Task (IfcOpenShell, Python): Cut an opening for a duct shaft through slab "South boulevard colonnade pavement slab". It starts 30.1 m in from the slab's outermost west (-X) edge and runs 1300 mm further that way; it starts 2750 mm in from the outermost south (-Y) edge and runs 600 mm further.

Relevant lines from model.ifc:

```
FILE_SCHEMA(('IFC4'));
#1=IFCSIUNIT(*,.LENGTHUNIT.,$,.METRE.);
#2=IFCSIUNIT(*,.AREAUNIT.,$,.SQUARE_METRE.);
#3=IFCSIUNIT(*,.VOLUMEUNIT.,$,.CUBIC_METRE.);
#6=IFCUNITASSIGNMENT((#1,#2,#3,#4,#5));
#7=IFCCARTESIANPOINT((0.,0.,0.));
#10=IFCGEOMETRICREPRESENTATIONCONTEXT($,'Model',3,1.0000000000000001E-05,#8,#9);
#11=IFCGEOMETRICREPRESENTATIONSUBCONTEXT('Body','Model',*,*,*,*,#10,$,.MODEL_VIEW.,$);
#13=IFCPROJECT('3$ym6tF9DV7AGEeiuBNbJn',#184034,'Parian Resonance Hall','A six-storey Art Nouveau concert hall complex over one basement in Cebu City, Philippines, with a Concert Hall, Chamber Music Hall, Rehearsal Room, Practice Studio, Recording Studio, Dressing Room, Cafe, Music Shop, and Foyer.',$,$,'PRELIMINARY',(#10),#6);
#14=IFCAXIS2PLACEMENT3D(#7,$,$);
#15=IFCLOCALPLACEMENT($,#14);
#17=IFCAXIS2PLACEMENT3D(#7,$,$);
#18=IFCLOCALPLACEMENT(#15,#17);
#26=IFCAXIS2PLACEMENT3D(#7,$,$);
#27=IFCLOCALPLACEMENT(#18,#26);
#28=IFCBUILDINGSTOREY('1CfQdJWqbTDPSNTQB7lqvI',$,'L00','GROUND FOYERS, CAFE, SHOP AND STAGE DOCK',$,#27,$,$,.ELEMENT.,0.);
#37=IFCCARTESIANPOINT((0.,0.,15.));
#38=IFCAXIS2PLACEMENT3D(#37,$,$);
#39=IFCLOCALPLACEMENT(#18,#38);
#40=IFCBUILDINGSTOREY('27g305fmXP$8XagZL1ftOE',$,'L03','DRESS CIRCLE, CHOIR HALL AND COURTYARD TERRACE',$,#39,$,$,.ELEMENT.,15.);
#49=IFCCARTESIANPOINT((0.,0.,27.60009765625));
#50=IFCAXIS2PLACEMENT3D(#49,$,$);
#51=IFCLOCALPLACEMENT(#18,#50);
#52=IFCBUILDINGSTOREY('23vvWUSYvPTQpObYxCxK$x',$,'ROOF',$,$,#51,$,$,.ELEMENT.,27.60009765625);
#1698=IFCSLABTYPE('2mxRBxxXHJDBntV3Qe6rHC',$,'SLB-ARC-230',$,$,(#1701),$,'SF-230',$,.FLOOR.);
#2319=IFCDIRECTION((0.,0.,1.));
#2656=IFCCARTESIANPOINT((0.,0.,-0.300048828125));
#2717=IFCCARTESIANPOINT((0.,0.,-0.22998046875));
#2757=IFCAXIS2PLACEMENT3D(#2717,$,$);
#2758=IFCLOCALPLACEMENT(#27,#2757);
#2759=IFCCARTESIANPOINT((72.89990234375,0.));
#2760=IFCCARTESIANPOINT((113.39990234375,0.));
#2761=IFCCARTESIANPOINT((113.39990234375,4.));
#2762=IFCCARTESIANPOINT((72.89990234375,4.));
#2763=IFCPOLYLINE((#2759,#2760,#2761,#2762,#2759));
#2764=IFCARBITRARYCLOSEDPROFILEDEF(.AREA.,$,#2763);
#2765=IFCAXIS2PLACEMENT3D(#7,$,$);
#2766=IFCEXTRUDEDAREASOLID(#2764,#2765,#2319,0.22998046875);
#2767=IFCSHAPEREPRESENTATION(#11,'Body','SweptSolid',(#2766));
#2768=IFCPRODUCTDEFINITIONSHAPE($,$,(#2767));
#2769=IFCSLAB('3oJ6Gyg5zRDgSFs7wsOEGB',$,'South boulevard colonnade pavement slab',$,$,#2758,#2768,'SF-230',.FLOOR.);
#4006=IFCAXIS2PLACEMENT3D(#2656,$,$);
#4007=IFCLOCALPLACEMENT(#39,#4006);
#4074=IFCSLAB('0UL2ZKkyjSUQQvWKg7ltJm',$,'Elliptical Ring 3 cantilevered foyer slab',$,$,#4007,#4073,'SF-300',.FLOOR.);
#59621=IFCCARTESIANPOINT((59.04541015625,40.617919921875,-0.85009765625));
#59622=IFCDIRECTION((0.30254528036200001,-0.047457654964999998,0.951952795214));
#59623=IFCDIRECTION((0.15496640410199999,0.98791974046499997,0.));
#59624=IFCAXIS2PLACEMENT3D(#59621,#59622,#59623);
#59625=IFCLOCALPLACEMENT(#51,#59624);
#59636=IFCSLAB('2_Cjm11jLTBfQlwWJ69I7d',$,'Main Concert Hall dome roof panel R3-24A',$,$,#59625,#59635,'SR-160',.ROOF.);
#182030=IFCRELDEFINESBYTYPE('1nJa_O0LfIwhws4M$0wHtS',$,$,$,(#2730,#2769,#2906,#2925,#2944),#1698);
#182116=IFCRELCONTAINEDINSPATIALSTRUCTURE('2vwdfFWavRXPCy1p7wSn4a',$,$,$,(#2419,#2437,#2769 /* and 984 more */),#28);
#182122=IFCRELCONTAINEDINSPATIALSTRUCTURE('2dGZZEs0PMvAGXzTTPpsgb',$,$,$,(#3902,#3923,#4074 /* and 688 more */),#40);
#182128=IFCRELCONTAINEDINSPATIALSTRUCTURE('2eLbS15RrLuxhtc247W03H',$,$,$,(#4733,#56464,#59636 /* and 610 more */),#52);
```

```python
import numpy as np
import ifcopenshell
import ifcopenshell.api.feature
import ifcopenshell.api.geometry
import ifcopenshell.api.root
import ifcopenshell.geom
import ifcopenshell.util.placement
import ifcopenshell.util.representation
import ifcopenshell.util.shape
import ifcopenshell.util.unit

model = ifcopenshell.open("model.ifc")
unit_scale = ifcopenshell.util.unit.calculate_unit_scale(model)
settings = ifcopenshell.geom.settings()


def volume(element):
    """Net volume in cubic metres, openings subtracted."""
    shape = ifcopenshell.geom.create_shape(settings, element)
    return ifcopenshell.util.shape.get_volume(shape.geometry)


slab = model.by_guid("3oJ6Gyg5zRDgSFs7wsOEGB")
before = volume(slab)

# Extent in the slab's own axes, in metres. The edges named are its -X and -Y sides.
slab_shape = ifcopenshell.geom.create_shape(settings, slab)
vertices = ifcopenshell.util.shape.get_vertices(slab_shape.geometry)
x_min, y_min, bottom = vertices.min(axis=0)
top = vertices[:, 2].max()

opening = ifcopenshell.api.root.create_entity(model, ifc_class="IfcOpeningElement", name="Duct shaft opening", predefined_type="OPENING")
context = ifcopenshell.util.representation.get_context(model, "Model", "Body", "MODEL_VIEW")
width, depth = 1.3, 0.6
outline = [(0.0, 0.0), (width, 0.0), (width, depth), (0.0, depth), (0.0, 0.0)]
# Overshoot both faces by 50 mm so the cut is clean.
shape = ifcopenshell.api.geometry.add_slab_representation(
    model, context=context, depth=top - bottom + 0.1, polyline=outline
)
ifcopenshell.api.geometry.assign_representation(model, product=opening, representation=shape)

matrix = ifcopenshell.util.placement.get_local_placement(slab.ObjectPlacement)
matrix[:, 3] = matrix @ np.append(np.array([x_min + 30.1, y_min + 2.75, bottom - 0.05]) / unit_scale, 1.0)
ifcopenshell.api.geometry.edit_object_placement(model, product=opening, matrix=matrix, is_si=False)
ifcopenshell.api.feature.add_feature(model, feature=opening, element=slab)

after = volume(slab)

print(f"slab volume {before:.3f} -> {after:.3f} m3")

model.write("model_edited.ifc")
```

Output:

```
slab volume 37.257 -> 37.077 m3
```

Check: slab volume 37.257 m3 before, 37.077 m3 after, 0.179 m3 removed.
